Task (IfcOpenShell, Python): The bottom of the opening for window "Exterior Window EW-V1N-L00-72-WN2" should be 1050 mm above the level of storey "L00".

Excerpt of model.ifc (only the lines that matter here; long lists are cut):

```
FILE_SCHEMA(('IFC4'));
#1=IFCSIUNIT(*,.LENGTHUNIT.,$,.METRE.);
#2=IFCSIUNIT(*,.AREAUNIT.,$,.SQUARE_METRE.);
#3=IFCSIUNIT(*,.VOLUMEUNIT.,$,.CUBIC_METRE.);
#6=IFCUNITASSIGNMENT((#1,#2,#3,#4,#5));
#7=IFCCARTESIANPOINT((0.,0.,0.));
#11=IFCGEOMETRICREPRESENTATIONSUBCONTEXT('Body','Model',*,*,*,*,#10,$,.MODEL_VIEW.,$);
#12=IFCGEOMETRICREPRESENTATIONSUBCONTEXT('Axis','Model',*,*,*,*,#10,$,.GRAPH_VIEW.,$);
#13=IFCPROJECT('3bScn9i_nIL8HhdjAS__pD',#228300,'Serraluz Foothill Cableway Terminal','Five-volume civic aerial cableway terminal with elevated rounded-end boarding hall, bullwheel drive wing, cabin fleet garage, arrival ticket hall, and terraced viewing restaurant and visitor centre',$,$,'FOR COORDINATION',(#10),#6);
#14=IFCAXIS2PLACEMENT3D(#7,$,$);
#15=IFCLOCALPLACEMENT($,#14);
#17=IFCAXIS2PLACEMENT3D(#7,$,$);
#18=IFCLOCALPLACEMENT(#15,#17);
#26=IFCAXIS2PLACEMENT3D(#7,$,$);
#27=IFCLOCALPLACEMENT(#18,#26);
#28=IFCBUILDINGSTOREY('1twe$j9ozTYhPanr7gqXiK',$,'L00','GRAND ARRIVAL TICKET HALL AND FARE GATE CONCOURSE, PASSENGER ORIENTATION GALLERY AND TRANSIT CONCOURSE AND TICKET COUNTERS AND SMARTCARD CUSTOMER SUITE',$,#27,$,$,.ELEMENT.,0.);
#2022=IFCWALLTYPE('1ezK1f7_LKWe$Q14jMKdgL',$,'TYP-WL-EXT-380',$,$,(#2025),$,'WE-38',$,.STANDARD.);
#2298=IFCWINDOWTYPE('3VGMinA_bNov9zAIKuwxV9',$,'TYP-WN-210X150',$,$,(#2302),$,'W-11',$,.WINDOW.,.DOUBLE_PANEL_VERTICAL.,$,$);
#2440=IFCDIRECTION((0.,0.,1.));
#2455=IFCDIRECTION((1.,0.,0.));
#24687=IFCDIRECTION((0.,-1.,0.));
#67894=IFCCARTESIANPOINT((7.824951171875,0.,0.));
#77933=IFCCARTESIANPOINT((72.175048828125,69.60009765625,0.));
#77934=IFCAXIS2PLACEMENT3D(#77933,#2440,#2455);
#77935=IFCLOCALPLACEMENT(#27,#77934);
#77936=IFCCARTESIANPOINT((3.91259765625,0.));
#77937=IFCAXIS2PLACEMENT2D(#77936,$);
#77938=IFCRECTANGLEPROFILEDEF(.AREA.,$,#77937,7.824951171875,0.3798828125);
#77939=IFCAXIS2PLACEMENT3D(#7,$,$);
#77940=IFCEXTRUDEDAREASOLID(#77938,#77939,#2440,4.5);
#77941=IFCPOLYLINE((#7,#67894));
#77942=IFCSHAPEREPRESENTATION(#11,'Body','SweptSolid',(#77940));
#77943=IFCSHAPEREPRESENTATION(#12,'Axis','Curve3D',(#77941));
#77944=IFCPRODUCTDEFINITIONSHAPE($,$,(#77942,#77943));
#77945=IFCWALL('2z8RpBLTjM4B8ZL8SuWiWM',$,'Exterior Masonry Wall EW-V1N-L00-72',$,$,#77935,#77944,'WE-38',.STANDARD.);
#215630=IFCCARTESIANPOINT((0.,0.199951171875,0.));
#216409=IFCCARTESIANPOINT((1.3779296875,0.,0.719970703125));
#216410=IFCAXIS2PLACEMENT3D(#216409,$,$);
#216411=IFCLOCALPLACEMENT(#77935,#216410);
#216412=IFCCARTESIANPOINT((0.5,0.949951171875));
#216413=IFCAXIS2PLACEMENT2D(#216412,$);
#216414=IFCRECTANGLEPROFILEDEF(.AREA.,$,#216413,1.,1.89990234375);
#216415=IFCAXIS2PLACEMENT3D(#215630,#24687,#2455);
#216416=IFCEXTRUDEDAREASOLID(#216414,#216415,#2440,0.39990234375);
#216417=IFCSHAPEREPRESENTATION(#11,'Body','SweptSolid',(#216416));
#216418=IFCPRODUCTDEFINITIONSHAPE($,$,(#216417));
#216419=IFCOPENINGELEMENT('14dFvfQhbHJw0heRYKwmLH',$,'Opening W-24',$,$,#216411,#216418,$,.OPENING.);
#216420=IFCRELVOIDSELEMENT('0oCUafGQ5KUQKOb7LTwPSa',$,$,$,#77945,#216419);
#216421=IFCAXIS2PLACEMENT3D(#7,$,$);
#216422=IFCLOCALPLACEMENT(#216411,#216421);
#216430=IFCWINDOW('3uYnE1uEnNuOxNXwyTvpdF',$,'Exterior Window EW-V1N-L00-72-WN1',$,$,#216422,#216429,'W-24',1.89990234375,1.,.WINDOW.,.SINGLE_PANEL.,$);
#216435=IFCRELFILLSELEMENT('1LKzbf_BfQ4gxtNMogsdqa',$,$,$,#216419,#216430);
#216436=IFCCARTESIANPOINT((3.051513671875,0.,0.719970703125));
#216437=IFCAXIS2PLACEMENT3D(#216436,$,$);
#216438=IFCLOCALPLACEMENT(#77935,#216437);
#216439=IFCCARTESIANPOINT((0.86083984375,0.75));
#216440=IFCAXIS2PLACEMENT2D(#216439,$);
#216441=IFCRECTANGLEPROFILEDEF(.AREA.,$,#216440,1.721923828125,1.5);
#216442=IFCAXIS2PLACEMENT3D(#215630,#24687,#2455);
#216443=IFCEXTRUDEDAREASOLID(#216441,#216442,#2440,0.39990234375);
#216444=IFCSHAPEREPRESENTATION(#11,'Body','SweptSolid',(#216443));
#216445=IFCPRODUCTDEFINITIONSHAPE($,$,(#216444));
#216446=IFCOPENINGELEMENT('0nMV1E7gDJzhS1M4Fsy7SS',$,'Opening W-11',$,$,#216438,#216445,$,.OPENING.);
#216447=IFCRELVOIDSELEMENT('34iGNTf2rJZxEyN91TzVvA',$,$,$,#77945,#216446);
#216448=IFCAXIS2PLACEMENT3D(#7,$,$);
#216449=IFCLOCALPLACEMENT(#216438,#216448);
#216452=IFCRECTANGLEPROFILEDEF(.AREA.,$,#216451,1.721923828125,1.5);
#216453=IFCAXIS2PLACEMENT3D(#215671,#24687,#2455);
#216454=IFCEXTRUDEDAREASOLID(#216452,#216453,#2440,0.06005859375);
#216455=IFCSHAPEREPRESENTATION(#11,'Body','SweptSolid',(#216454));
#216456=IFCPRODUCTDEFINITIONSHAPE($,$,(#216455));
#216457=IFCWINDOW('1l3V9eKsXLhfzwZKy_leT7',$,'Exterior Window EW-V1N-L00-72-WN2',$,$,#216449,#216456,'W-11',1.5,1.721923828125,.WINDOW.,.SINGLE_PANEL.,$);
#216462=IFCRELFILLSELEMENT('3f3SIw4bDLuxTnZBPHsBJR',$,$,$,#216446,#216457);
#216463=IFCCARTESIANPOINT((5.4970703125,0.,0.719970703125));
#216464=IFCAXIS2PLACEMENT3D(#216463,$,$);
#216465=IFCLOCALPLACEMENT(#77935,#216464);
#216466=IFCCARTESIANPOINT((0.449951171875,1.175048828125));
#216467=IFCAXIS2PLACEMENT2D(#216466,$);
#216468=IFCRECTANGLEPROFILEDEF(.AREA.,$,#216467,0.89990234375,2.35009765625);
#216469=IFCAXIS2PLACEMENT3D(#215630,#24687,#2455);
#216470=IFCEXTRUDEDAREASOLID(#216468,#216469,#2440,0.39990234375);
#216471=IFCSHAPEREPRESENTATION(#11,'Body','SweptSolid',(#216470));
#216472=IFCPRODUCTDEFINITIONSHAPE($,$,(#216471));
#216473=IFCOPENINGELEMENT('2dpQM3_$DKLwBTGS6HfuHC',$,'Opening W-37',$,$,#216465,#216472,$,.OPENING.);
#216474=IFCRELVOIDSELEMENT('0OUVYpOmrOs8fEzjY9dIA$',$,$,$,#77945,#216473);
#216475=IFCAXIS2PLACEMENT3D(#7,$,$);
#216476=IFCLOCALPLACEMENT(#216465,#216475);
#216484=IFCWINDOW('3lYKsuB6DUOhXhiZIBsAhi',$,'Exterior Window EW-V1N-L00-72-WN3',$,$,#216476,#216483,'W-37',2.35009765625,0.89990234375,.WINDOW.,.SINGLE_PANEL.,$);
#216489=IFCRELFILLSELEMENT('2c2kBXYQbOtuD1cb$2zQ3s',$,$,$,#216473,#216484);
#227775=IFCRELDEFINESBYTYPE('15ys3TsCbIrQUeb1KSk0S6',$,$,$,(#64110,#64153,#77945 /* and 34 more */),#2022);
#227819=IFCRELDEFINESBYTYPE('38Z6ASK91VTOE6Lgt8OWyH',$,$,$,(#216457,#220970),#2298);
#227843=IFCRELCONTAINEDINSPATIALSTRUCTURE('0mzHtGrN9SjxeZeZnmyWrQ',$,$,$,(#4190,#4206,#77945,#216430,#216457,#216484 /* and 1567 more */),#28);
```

```python
import numpy as np
import ifcopenshell
import ifcopenshell.api.geometry
import ifcopenshell.geom
import ifcopenshell.util.element
import ifcopenshell.util.placement
import ifcopenshell.util.shape
import ifcopenshell.util.unit

model = ifcopenshell.open("model.ifc")
unit_scale = ifcopenshell.util.unit.calculate_unit_scale(model)

window = model.by_guid("1l3V9eKsXLhfzwZKy_leT7")
opening = window.FillsVoids[0].RelatingOpeningElement
storey = ifcopenshell.util.element.get_container(window, ifc_class="IfcBuildingStorey")
level = ifcopenshell.util.placement.get_local_placement(storey.ObjectPlacement)[2, 3]

# The opening's origin need not be at the sill, so measure its lowest point.
shape = ifcopenshell.geom.create_shape(ifcopenshell.geom.settings(), opening)
bottom = ifcopenshell.util.shape.get_shape_bottom_elevation(shape, shape.geometry) / unit_scale
dz = level + 1.05 / unit_scale - bottom

shift = np.array([0.0, 0.0, dz])
# The window is placed relative to its opening, so it follows when the opening moves.
matrix = ifcopenshell.util.placement.get_local_placement(opening.ObjectPlacement)
matrix[:3, 3] += shift
ifcopenshell.api.geometry.edit_object_placement(
    model, product=opening, matrix=matrix, is_si=False, should_transform_children=True
)

print(f"moved by {dz * unit_scale:+.3f} m")

model.write("model_v2.ifc")
```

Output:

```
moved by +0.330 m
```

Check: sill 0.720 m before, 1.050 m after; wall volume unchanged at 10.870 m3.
